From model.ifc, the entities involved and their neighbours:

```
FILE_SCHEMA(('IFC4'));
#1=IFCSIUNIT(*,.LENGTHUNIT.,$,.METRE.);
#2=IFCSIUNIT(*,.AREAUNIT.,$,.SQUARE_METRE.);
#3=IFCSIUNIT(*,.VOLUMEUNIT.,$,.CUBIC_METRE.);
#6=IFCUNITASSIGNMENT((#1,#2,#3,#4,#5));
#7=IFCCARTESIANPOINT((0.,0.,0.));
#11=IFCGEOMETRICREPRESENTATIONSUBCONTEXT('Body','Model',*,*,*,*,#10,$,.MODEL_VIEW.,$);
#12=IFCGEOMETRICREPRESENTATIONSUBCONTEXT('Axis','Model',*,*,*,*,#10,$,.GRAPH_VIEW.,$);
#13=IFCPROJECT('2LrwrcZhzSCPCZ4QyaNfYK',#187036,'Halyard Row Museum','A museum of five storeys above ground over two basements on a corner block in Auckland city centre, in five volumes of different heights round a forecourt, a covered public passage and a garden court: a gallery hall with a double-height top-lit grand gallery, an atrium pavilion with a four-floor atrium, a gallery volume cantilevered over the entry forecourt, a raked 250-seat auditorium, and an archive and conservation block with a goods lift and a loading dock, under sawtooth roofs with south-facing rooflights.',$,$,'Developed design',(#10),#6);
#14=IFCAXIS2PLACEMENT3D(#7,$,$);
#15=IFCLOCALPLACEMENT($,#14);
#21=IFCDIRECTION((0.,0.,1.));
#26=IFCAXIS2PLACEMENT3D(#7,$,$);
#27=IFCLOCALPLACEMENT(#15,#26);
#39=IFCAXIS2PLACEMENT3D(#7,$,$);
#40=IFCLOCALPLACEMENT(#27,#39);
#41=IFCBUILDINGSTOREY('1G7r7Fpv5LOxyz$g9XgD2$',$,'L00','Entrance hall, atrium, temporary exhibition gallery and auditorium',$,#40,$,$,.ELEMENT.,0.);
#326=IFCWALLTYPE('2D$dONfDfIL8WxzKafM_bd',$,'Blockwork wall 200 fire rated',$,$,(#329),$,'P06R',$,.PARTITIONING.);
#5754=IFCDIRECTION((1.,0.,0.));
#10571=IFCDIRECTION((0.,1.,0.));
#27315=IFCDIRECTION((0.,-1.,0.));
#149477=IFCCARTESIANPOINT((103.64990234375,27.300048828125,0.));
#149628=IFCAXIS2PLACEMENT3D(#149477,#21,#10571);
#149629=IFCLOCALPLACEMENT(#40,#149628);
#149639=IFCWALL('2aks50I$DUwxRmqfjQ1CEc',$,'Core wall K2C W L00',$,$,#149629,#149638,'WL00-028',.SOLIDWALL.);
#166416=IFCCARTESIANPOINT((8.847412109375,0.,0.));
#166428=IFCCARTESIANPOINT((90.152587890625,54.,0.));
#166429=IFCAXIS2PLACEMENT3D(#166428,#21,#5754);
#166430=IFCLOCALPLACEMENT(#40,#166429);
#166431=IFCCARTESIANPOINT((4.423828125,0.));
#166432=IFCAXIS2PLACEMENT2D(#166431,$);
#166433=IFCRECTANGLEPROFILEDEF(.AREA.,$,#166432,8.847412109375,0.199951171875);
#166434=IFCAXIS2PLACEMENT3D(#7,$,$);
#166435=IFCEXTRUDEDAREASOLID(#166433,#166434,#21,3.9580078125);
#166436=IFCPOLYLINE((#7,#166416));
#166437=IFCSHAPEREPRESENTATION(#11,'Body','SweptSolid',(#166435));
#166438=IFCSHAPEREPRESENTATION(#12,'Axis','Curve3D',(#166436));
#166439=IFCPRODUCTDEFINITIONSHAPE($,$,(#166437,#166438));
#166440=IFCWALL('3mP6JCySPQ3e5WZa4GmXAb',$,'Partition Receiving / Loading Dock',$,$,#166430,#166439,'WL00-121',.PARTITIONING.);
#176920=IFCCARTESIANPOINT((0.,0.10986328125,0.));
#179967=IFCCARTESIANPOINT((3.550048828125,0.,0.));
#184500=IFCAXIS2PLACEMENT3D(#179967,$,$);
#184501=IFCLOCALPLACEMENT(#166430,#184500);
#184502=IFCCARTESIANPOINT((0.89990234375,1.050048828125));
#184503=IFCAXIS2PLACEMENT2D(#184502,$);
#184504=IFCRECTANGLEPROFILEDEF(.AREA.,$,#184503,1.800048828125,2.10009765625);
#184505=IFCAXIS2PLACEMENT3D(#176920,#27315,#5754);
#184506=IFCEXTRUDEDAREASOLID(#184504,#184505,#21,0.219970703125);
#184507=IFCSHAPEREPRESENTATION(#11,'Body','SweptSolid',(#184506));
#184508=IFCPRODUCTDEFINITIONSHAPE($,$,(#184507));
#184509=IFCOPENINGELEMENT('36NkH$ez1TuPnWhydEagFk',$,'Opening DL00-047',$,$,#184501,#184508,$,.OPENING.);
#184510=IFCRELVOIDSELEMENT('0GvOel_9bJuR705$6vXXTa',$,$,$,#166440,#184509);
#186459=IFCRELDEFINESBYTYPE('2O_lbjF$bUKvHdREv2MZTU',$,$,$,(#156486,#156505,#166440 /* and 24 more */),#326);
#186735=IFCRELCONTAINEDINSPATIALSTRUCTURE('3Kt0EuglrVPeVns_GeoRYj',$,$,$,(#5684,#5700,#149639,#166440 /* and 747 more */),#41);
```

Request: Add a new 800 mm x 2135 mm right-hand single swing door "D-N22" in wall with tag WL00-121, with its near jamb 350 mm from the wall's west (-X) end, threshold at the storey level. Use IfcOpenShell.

```python
import numpy as np
import ifcopenshell
import ifcopenshell.api.feature
import ifcopenshell.api.geometry
import ifcopenshell.api.root
import ifcopenshell.api.spatial
import ifcopenshell.geom
import ifcopenshell.util.element
import ifcopenshell.util.placement
import ifcopenshell.util.representation
import ifcopenshell.util.shape
import ifcopenshell.util.unit

model = ifcopenshell.open("model.ifc")
unit_scale = ifcopenshell.util.unit.calculate_unit_scale(model)
settings = ifcopenshell.geom.settings()


def volume(element):
    """Net volume in cubic metres, openings subtracted."""
    shape = ifcopenshell.geom.create_shape(settings, element)
    return ifcopenshell.util.shape.get_volume(shape.geometry)


wall = model.by_guid("3mP6JCySPQ3e5WZa4GmXAb")
storey = ifcopenshell.util.element.get_container(wall, ifc_class="IfcBuildingStorey")
context = ifcopenshell.util.representation.get_context(model, "Model", "Body", "MODEL_VIEW")
before = volume(wall)

width, height, from_end, sill = 0.8, 2.135, 0.35, 0.0  # metres

# The wall runs along its own X axis, and the end named is its -X end.
wall_shape = ifcopenshell.geom.create_shape(settings, wall)
x, y, z = ifcopenshell.util.shape.get_vertices(wall_shape.geometry).T
start = x.min() + from_end
face, thickness = float(y.min()), float(y.max() - y.min())
wall_matrix = ifcopenshell.util.placement.get_local_placement(wall.ObjectPlacement)
level = ifcopenshell.util.placement.get_local_placement(storey.ObjectPlacement)[2, 3]


def in_wall(x, y):
    """Placement at x, y metres in the wall's axes, at sill height."""
    matrix = wall_matrix.copy()
    matrix[:, 3] = wall_matrix @ np.array([x / unit_scale, y / unit_scale, 0.0, 1.0])
    matrix[2, 3] = level + sill / unit_scale
    return matrix


# Opening: a box that overshoots both wall faces by 50 mm.
opening = ifcopenshell.api.root.create_entity(model, ifc_class="IfcOpeningElement", predefined_type="OPENING")
box = ifcopenshell.api.geometry.add_wall_representation(
    model, context=context, length=width, height=height, thickness=thickness + 0.1
)
ifcopenshell.api.geometry.assign_representation(model, product=opening, representation=box)
ifcopenshell.api.geometry.edit_object_placement(model, product=opening, matrix=in_wall(start, face - 0.05), is_si=False)
ifcopenshell.api.feature.add_feature(model, feature=opening, element=wall)

door = ifcopenshell.api.root.create_entity(model, ifc_class="IfcDoor", name="D-N22", predefined_type="DOOR")
door.OverallWidth, door.OverallHeight = width / unit_scale, height / unit_scale
door.OperationType = "SINGLE_SWING_RIGHT"
body = ifcopenshell.api.geometry.add_door_representation(
    model,
    context=context,
    overall_width=door.OverallWidth,
    overall_height=door.OverallHeight,
    operation_type="SINGLE_SWING_RIGHT",
    lining_properties={"LiningDepth": thickness / unit_scale, "ThresholdDepth": thickness / unit_scale},
)
ifcopenshell.api.geometry.assign_representation(model, product=door, representation=body)
ifcopenshell.api.spatial.assign_container(model, products=[door], relating_structure=storey)
ifcopenshell.api.feature.add_filling(model, opening=opening, element=door)

# The lining spans the wall, so the door starts at the wall face.
ifcopenshell.api.geometry.edit_object_placement(model, product=door, matrix=in_wall(start, face), is_si=False)

after = volume(wall)

print(f"wall volume {before:.3f} -> {after:.3f} m3")

model.write("model-out.ifc")
```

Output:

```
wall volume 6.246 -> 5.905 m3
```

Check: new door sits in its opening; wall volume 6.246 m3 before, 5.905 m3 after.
